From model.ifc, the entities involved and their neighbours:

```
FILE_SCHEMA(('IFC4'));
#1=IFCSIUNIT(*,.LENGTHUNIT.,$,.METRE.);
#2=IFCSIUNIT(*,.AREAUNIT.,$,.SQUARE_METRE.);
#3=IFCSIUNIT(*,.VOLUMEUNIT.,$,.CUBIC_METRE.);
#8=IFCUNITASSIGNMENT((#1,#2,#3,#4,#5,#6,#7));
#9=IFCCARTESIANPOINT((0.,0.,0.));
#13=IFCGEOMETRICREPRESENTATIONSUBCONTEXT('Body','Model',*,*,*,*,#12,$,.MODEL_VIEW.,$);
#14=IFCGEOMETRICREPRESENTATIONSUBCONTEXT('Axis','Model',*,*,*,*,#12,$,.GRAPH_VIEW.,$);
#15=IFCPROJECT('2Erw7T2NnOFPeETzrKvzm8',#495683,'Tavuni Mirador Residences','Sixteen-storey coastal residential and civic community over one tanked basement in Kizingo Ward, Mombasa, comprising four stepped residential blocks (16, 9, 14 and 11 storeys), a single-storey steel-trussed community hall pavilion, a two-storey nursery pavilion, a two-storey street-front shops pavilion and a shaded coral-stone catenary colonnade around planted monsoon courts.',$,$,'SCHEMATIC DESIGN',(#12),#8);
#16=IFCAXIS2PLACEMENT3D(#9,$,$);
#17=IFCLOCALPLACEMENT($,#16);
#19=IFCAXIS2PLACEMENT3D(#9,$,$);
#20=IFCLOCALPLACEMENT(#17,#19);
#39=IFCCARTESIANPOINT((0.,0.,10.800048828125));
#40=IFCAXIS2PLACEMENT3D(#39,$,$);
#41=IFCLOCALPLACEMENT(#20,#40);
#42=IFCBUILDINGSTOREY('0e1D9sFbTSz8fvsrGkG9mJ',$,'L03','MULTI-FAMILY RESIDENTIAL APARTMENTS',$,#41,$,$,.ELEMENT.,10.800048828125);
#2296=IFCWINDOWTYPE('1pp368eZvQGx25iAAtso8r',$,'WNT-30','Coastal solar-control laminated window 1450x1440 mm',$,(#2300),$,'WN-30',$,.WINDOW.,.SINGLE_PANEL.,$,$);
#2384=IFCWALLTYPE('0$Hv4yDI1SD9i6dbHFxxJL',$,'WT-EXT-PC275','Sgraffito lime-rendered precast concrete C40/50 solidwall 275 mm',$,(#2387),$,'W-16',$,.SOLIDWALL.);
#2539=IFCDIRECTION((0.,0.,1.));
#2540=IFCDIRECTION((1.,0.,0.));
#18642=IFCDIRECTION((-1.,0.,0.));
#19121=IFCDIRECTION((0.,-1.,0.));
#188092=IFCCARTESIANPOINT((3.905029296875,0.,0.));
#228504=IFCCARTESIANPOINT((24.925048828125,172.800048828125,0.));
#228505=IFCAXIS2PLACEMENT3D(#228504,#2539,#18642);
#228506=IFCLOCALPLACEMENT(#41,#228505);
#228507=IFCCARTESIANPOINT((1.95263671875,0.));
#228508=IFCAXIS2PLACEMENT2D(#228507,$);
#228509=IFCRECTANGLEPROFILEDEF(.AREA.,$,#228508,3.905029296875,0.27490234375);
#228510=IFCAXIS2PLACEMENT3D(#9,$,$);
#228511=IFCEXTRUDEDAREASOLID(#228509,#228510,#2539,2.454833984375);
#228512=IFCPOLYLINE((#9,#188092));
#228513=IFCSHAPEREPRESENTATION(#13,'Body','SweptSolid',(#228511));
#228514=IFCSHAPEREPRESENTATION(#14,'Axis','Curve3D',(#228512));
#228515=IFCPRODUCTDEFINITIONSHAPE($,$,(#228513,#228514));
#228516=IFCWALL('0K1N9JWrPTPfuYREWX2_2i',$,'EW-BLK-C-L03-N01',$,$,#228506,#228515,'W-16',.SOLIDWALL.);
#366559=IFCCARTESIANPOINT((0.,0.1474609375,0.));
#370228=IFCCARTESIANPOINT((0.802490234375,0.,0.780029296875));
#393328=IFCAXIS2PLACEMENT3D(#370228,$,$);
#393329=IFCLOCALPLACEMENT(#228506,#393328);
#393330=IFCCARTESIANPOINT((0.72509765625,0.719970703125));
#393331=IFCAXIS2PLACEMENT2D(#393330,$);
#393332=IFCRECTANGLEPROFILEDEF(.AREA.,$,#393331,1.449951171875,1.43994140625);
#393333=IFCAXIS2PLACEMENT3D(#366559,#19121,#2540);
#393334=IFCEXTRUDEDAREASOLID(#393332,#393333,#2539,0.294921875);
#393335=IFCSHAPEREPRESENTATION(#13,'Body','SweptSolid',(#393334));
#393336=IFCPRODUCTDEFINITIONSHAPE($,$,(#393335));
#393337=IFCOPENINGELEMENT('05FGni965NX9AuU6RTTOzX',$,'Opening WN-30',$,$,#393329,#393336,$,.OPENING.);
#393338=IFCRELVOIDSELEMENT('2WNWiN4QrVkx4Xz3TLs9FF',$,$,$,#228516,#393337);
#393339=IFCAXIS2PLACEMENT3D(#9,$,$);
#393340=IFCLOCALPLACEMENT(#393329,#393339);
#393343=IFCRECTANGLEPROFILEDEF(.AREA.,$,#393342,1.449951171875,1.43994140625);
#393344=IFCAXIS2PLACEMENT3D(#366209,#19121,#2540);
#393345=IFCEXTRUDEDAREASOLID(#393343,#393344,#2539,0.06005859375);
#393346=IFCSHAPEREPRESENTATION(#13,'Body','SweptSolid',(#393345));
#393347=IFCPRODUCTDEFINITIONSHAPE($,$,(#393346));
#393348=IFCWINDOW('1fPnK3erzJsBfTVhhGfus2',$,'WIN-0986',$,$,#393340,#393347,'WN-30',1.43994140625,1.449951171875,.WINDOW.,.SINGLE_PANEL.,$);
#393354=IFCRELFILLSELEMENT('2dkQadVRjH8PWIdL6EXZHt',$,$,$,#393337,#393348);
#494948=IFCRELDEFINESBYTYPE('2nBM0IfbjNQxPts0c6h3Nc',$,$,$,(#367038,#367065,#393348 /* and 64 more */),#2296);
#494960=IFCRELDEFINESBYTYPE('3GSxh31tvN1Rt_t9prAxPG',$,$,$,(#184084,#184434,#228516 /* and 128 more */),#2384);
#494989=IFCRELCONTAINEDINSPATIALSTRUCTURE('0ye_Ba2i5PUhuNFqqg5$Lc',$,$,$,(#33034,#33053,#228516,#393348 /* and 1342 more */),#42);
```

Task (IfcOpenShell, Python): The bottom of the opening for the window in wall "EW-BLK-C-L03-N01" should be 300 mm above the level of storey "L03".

```python
import numpy as np
import ifcopenshell
import ifcopenshell.api.geometry
import ifcopenshell.geom
import ifcopenshell.util.element
import ifcopenshell.util.placement
import ifcopenshell.util.shape
import ifcopenshell.util.unit

model = ifcopenshell.open("model.ifc")
unit_scale = ifcopenshell.util.unit.calculate_unit_scale(model)

window = model.by_id(393348)
opening = window.FillsVoids[0].RelatingOpeningElement
storey = ifcopenshell.util.element.get_container(window, ifc_class="IfcBuildingStorey")
level = ifcopenshell.util.placement.get_local_placement(storey.ObjectPlacement)[2, 3]

# The opening's origin need not be at the sill, so measure its lowest point.
shape = ifcopenshell.geom.create_shape(ifcopenshell.geom.settings(), opening)
bottom = ifcopenshell.util.shape.get_shape_bottom_elevation(shape, shape.geometry) / unit_scale
dz = level + 0.3 - bottom

shift = np.array([0.0, 0.0, dz])
# The window is placed relative to its opening, so it follows when the opening moves.
matrix = ifcopenshell.util.placement.get_local_placement(opening.ObjectPlacement)
matrix[:3, 3] += shift
ifcopenshell.api.geometry.edit_object_placement(
    model, product=opening, matrix=matrix, is_si=False, should_transform_children=True
)

print(f"moved by {dz * unit_scale:+.3f} m")

model.write("model-out.ifc")
```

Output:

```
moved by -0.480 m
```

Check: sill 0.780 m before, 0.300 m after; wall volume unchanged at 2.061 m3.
